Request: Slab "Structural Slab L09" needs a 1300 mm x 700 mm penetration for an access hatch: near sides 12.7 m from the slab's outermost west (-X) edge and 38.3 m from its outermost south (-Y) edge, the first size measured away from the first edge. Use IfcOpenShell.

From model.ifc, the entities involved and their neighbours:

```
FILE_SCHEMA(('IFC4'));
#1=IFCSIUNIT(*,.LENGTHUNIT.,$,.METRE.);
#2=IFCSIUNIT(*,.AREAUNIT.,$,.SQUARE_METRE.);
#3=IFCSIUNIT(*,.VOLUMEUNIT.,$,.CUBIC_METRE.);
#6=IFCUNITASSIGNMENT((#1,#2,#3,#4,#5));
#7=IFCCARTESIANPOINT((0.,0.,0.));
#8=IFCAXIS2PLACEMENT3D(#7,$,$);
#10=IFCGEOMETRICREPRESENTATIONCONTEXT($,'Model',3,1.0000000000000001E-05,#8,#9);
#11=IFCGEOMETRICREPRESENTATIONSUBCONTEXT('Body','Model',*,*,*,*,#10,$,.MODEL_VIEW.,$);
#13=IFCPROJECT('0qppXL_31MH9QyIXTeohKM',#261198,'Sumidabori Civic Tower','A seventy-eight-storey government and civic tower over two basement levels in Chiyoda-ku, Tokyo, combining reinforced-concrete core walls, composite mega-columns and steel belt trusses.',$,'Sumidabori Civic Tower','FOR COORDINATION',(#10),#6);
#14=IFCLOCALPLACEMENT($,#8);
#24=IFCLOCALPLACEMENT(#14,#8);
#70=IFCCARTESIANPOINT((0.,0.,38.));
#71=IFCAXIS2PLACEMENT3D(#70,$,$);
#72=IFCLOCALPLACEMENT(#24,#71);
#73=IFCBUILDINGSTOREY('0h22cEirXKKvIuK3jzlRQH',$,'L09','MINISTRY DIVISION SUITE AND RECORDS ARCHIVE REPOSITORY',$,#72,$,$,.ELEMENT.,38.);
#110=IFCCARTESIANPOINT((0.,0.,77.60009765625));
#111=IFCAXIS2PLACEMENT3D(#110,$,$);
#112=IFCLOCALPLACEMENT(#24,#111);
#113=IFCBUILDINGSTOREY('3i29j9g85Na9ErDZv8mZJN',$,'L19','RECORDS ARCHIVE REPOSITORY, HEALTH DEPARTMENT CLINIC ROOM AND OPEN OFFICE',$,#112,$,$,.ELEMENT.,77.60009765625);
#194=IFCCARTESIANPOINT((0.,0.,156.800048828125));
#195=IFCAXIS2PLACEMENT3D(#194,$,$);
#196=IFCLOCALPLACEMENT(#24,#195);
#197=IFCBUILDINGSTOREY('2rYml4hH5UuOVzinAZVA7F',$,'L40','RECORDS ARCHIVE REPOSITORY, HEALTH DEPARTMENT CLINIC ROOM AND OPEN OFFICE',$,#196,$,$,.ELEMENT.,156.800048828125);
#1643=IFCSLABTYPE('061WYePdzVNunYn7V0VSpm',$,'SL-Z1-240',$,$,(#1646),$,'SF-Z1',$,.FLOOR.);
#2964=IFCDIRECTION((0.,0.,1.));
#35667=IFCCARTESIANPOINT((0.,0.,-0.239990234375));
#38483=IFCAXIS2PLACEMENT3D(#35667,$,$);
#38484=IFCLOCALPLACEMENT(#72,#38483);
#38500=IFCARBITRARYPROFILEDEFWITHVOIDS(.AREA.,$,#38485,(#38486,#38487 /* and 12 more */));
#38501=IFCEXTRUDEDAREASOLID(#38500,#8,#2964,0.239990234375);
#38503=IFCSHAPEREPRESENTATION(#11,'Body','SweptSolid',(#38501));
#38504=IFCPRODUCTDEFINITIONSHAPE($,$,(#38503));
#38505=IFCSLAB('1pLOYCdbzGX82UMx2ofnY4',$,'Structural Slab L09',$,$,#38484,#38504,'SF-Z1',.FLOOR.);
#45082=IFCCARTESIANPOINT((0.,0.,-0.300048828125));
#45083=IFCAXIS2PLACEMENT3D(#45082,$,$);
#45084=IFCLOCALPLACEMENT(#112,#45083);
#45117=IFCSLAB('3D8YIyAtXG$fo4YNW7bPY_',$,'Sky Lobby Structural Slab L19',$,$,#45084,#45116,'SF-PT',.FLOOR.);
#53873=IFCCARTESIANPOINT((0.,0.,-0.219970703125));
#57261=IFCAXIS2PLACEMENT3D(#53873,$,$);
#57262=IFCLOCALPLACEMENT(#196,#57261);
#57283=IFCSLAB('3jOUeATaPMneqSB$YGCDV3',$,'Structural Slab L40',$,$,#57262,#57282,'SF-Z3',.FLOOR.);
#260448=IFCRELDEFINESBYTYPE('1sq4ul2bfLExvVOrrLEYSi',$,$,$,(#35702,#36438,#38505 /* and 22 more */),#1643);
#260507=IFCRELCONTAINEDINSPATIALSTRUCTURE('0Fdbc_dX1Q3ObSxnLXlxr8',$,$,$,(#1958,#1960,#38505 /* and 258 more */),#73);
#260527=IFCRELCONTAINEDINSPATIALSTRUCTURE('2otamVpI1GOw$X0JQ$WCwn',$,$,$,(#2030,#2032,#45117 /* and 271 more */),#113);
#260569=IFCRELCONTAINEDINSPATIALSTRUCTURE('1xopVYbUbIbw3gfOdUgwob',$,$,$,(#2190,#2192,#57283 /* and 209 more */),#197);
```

```python
import numpy as np
import ifcopenshell
import ifcopenshell.api.feature
import ifcopenshell.api.geometry
import ifcopenshell.api.root
import ifcopenshell.geom
import ifcopenshell.util.placement
import ifcopenshell.util.representation
import ifcopenshell.util.shape
import ifcopenshell.util.unit

model = ifcopenshell.open("model.ifc")
unit_scale = ifcopenshell.util.unit.calculate_unit_scale(model)
settings = ifcopenshell.geom.settings()


def volume(element):
    """Net volume in cubic metres, openings subtracted."""
    shape = ifcopenshell.geom.create_shape(settings, element)
    return ifcopenshell.util.shape.get_volume(shape.geometry)


slab = model.by_guid("1pLOYCdbzGX82UMx2ofnY4")
before = volume(slab)

# Extent in the slab's own axes, in metres. The edges named are its -X and -Y sides.
slab_shape = ifcopenshell.geom.create_shape(settings, slab)
vertices = ifcopenshell.util.shape.get_vertices(slab_shape.geometry)
x_min, y_min, bottom = vertices.min(axis=0)
top = vertices[:, 2].max()

opening = ifcopenshell.api.root.create_entity(model, ifc_class="IfcOpeningElement", name="Access hatch opening", predefined_type="OPENING")
context = ifcopenshell.util.representation.get_context(model, "Model", "Body", "MODEL_VIEW")
width, depth = 1.3, 0.7
outline = [(0.0, 0.0), (width, 0.0), (width, depth), (0.0, depth), (0.0, 0.0)]
# Overshoot both faces by 50 mm so the cut is clean.
shape = ifcopenshell.api.geometry.add_slab_representation(
    model, context=context, depth=top - bottom + 0.1, polyline=outline
)
ifcopenshell.api.geometry.assign_representation(model, product=opening, representation=shape)

matrix = ifcopenshell.util.placement.get_local_placement(slab.ObjectPlacement)
matrix[:, 3] = matrix @ np.append(np.array([x_min + 12.7, y_min + 38.3, bottom - 0.05]) / unit_scale, 1.0)
ifcopenshell.api.geometry.edit_object_placement(model, product=opening, matrix=matrix, is_si=False)
ifcopenshell.api.feature.add_feature(model, feature=opening, element=slab)

after = volume(slab)

print(f"slab volume {before:.3f} -> {after:.3f} m3")

model.write("model_edited.ifc")
```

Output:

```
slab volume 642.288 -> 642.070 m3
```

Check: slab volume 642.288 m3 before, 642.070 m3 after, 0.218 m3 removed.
